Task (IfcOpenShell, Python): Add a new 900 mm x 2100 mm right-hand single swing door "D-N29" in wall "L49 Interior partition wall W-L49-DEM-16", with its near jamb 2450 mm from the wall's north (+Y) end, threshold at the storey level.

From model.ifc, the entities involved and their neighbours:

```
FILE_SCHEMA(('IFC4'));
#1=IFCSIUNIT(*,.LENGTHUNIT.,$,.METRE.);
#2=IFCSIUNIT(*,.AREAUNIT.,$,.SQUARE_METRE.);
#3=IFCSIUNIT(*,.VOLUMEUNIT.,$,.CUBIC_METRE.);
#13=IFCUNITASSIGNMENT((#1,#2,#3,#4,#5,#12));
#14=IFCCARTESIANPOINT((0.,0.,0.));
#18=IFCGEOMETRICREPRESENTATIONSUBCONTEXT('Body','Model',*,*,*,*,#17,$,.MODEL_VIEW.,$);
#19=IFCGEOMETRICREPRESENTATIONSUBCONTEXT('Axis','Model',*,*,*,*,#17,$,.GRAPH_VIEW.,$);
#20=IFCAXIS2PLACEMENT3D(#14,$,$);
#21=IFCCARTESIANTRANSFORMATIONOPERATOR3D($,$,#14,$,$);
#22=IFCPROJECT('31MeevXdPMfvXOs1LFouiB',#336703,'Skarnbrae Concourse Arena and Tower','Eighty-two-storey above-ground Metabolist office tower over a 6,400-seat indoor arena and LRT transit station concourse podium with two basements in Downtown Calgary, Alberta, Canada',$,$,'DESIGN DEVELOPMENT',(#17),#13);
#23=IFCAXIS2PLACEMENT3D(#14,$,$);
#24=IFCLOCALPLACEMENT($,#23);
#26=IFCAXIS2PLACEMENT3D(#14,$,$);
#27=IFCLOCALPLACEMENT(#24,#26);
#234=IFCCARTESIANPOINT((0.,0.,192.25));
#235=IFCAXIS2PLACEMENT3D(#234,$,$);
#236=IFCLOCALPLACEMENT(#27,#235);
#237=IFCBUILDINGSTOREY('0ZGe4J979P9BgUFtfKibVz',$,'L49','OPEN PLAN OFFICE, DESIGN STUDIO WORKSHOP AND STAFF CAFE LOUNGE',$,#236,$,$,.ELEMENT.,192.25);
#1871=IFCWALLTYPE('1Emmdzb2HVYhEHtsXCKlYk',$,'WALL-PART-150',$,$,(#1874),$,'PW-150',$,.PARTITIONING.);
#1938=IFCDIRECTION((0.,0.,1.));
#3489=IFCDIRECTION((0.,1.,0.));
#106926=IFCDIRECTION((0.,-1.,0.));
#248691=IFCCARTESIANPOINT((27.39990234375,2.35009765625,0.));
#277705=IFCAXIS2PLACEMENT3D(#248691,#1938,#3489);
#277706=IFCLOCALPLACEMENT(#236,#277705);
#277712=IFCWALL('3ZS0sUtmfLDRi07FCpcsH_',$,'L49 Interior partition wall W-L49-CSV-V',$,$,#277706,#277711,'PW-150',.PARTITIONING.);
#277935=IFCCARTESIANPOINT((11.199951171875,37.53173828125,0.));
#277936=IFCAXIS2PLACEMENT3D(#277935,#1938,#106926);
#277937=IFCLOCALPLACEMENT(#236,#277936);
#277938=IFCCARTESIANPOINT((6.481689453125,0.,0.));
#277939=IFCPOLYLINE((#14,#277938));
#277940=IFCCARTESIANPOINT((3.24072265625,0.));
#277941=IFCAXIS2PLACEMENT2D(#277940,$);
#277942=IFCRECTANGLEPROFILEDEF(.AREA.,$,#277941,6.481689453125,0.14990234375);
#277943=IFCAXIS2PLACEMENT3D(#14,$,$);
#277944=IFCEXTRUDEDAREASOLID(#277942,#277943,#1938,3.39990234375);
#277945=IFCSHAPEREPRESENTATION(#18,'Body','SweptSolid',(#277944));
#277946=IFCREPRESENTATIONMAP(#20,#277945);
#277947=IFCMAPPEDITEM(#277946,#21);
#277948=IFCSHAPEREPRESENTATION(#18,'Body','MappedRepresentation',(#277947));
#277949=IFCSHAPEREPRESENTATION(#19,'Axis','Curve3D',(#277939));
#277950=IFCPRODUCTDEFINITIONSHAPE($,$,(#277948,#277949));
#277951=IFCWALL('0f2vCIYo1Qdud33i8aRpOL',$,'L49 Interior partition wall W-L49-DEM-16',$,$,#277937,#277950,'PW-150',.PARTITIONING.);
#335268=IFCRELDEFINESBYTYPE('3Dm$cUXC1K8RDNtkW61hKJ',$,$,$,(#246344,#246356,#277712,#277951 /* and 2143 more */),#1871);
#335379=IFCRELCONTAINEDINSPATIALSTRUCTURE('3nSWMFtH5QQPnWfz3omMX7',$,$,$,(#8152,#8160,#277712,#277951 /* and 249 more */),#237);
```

```python
import numpy as np
import ifcopenshell
import ifcopenshell.api.feature
import ifcopenshell.api.geometry
import ifcopenshell.api.root
import ifcopenshell.api.spatial
import ifcopenshell.geom
import ifcopenshell.util.element
import ifcopenshell.util.placement
import ifcopenshell.util.representation
import ifcopenshell.util.shape
import ifcopenshell.util.unit

model = ifcopenshell.open("model.ifc")
unit_scale = ifcopenshell.util.unit.calculate_unit_scale(model)
settings = ifcopenshell.geom.settings()


def volume(element):
    """Net volume in cubic metres, openings subtracted."""
    shape = ifcopenshell.geom.create_shape(settings, element)
    return ifcopenshell.util.shape.get_volume(shape.geometry)


wall = model.by_guid("0f2vCIYo1Qdud33i8aRpOL")
storey = ifcopenshell.util.element.get_container(wall, ifc_class="IfcBuildingStorey")
context = ifcopenshell.util.representation.get_context(model, "Model", "Body", "MODEL_VIEW")
before = volume(wall)

width, height, from_end, sill = 0.9, 2.1, 2.45, 0.0  # metres

# The wall runs along its own X axis, and the end named is its -X end.
wall_shape = ifcopenshell.geom.create_shape(settings, wall)
x, y, z = ifcopenshell.util.shape.get_vertices(wall_shape.geometry).T
start = x.min() + from_end
face, thickness = float(y.min()), float(y.max() - y.min())
wall_matrix = ifcopenshell.util.placement.get_local_placement(wall.ObjectPlacement)
level = ifcopenshell.util.placement.get_local_placement(storey.ObjectPlacement)[2, 3]


def in_wall(x, y):
    """Placement at x, y metres in the wall's axes, at sill height."""
    matrix = wall_matrix.copy()
    matrix[:, 3] = wall_matrix @ np.array([x / unit_scale, y / unit_scale, 0.0, 1.0])
    matrix[2, 3] = level + sill / unit_scale
    return matrix


# Opening: a box that overshoots both wall faces by 50 mm.
opening = ifcopenshell.api.root.create_entity(model, ifc_class="IfcOpeningElement", predefined_type="OPENING")
box = ifcopenshell.api.geometry.add_wall_representation(
    model, context=context, length=width, height=height, thickness=thickness + 0.1
)
ifcopenshell.api.geometry.assign_representation(model, product=opening, representation=box)
ifcopenshell.api.geometry.edit_object_placement(model, product=opening, matrix=in_wall(start, face - 0.05), is_si=False)
ifcopenshell.api.feature.add_feature(model, feature=opening, element=wall)

door = ifcopenshell.api.root.create_entity(model, ifc_class="IfcDoor", name="D-N29", predefined_type="DOOR")
door.OverallWidth, door.OverallHeight = width / unit_scale, height / unit_scale
door.OperationType = "SINGLE_SWING_RIGHT"
body = ifcopenshell.api.geometry.add_door_representation(
    model,
    context=context,
    overall_width=door.OverallWidth,
    overall_height=door.OverallHeight,
    operation_type="SINGLE_SWING_RIGHT",
    lining_properties={"LiningDepth": thickness / unit_scale, "ThresholdDepth": thickness / unit_scale},
)
ifcopenshell.api.geometry.assign_representation(model, product=door, representation=body)
ifcopenshell.api.spatial.assign_container(model, products=[door], relating_structure=storey)
ifcopenshell.api.feature.add_filling(model, opening=opening, element=door)

# The lining spans the wall, so the door starts at the wall face.
ifcopenshell.api.geometry.edit_object_placement(model, product=door, matrix=in_wall(start, face), is_si=False)

after = volume(wall)

print(f"wall volume {before:.3f} -> {after:.3f} m3")

model.write("model_rev.ifc")
```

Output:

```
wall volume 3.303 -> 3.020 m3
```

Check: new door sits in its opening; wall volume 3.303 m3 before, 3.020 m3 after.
